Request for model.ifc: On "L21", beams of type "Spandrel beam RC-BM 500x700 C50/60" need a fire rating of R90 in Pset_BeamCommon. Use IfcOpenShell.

First a look at what the model holds.

```python
import ifcopenshell
import ifcopenshell.util.element

model = ifcopenshell.open("model.ifc")
print(model.schema)
storey = next(s for s in model.by_type("IfcBuildingStorey") if s.Name == "L21")
beams = [e for e in ifcopenshell.util.element.get_decomposition(storey) if e.is_a("IfcBeam")]
seen = {}
for e in beams:
    element_type = ifcopenshell.util.element.get_type(e)
    key = (element_type.Name if element_type != e and element_type else None, ifcopenshell.util.element.get_pset(e, "Pset_BeamCommon", "FireRating"))
    seen[key] = seen.get(key, 0) + 1
for (name, value), count in sorted(seen.items(), key=str):
    print(count, "x", name, "|", value)
```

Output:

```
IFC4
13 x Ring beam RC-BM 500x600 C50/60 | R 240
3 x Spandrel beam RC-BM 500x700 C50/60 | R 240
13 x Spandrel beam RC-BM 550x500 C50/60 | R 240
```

```python
import ifcopenshell
import ifcopenshell.api.pset
import ifcopenshell.util.element

model = ifcopenshell.open("model.ifc")

storey = next(s for s in model.by_type("IfcBuildingStorey") if s.Name == "L21")
beams = [e for e in ifcopenshell.util.element.get_decomposition(storey) if e.is_a("IfcBeam")]

count = 0
for e in beams:
    element_type = ifcopenshell.util.element.get_type(e)
    if element_type in (None, e) or element_type.Name != "Spandrel beam RC-BM 500x700 C50/60":
        continue
    found = ifcopenshell.util.element.get_pset(e, "Pset_BeamCommon", should_inherit=False)
    if found:
        pset = model.by_id(found["id"])
        if len(ifcopenshell.util.element.get_elements_by_pset(pset)) > 1:
            pset = ifcopenshell.api.pset.unshare_pset(model, products=[e], pset=pset)[0]
    else:
        pset = ifcopenshell.api.pset.add_pset(model, product=e, name="Pset_BeamCommon")
    ifcopenshell.api.pset.edit_pset(model, pset=pset, properties={"FireRating": "R90"})
    count += 1

print(count, "beams updated")

model.write("model-out.ifc")
```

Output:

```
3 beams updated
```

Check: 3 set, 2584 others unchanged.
